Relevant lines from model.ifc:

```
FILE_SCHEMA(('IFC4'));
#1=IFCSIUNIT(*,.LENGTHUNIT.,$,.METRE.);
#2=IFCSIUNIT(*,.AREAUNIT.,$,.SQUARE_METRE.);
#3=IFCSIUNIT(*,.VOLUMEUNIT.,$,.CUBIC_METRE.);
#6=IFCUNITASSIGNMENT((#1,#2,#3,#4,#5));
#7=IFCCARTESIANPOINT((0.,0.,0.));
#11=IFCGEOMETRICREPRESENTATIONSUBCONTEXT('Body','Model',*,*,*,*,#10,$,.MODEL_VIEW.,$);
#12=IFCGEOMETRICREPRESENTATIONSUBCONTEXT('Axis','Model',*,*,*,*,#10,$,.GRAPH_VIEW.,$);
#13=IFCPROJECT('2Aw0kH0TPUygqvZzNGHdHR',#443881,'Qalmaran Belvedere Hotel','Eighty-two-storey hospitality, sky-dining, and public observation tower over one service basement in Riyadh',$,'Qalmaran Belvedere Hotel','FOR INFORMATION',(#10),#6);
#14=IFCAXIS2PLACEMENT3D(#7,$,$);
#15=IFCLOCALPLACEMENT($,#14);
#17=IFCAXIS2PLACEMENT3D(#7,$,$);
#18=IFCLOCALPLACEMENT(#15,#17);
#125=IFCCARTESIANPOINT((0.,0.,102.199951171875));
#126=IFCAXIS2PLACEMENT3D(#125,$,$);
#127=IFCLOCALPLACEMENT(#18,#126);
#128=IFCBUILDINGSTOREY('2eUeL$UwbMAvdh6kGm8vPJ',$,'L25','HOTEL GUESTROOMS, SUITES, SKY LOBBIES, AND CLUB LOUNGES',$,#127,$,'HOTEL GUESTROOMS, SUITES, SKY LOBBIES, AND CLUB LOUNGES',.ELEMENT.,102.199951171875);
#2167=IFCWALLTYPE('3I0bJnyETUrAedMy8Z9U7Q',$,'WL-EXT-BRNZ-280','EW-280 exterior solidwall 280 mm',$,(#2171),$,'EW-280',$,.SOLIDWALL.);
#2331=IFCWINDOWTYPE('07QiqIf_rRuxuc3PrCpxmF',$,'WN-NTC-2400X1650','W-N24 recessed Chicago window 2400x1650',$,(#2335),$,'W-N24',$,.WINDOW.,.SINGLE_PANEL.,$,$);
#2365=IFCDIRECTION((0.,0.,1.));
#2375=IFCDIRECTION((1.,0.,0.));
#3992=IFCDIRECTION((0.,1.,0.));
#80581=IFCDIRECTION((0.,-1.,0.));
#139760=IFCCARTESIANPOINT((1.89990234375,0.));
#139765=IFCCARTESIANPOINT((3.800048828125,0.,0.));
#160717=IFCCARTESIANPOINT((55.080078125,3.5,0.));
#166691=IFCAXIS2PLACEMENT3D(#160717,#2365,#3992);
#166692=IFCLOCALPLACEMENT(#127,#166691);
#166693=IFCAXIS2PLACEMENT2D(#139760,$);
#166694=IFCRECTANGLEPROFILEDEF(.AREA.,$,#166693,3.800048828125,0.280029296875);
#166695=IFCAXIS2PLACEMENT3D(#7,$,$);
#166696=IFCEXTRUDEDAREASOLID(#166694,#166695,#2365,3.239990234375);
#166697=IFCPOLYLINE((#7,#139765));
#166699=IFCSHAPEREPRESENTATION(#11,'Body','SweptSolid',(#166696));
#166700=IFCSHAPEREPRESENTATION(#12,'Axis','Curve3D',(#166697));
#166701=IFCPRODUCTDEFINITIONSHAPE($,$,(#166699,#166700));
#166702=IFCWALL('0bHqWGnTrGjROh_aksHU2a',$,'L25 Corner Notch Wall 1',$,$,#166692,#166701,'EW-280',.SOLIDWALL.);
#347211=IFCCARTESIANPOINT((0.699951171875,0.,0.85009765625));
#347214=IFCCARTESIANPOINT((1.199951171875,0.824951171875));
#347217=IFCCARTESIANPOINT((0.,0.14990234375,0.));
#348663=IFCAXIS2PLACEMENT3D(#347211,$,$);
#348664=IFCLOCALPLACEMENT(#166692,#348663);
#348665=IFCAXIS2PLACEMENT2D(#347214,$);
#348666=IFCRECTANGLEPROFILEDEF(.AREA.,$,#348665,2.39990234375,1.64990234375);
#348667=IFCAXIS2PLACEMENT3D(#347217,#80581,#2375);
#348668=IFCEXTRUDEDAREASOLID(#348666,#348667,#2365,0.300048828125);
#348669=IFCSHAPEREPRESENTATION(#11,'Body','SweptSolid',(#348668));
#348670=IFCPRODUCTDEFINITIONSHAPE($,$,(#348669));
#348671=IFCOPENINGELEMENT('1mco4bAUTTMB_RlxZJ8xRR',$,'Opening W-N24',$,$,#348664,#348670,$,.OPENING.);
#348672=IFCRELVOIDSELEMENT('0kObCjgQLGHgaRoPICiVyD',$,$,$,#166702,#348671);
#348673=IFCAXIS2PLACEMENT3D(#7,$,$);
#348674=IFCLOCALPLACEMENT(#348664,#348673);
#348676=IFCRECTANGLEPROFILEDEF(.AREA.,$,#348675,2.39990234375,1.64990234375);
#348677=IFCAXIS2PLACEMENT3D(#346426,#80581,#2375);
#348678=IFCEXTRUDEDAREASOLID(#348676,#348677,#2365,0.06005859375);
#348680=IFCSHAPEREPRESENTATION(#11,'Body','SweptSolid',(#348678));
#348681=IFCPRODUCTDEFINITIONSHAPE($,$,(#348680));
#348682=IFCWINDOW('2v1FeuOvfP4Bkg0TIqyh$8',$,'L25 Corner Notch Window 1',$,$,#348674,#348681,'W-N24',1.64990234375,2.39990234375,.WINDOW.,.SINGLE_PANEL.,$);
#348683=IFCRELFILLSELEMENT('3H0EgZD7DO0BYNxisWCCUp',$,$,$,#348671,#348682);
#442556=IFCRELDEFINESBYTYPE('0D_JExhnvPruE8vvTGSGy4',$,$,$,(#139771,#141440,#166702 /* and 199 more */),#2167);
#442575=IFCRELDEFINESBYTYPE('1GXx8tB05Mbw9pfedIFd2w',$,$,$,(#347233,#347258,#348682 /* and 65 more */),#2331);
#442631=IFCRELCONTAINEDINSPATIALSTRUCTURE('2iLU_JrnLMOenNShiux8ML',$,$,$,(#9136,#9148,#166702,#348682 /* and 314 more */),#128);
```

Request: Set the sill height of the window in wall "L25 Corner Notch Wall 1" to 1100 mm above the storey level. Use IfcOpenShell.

```python
import numpy as np
import ifcopenshell
import ifcopenshell.api.geometry
import ifcopenshell.geom
import ifcopenshell.util.element
import ifcopenshell.util.placement
import ifcopenshell.util.shape
import ifcopenshell.util.unit

model = ifcopenshell.open("model.ifc")
unit_scale = ifcopenshell.util.unit.calculate_unit_scale(model)

window = model.by_guid("2v1FeuOvfP4Bkg0TIqyh$8")
opening = window.FillsVoids[0].RelatingOpeningElement
storey = ifcopenshell.util.element.get_container(window, ifc_class="IfcBuildingStorey")
level = ifcopenshell.util.placement.get_local_placement(storey.ObjectPlacement)[2, 3]

# The opening's origin need not be at the sill, so measure its lowest point.
shape = ifcopenshell.geom.create_shape(ifcopenshell.geom.settings(), opening)
bottom = ifcopenshell.util.shape.get_shape_bottom_elevation(shape, shape.geometry) / unit_scale
dz = level + 1.1 - bottom

shift = np.array([0.0, 0.0, dz])
# The window is placed relative to its opening, so it follows when the opening moves.
matrix = ifcopenshell.util.placement.get_local_placement(opening.ObjectPlacement)
matrix[:3, 3] += shift
ifcopenshell.api.geometry.edit_object_placement(
    model, product=opening, matrix=matrix, is_si=False, should_transform_children=True
)

print(f"moved by {dz * unit_scale:+.3f} m")

model.write("model_rev.ifc")
```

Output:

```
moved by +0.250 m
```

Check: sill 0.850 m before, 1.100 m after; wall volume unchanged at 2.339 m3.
